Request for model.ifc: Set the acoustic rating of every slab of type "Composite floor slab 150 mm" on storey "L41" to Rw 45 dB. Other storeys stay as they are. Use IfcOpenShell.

First a look at what the model holds.

```python
import ifcopenshell
import ifcopenshell.util.element

model = ifcopenshell.open("model.ifc")
print(model.schema)
storey = next(s for s in model.by_type("IfcBuildingStorey") if s.Name == "L41")
slabs = [e for e in ifcopenshell.util.element.get_decomposition(storey) if e.is_a("IfcSlab")]
seen = {}
for e in slabs:
    element_type = ifcopenshell.util.element.get_type(e)
    key = (element_type.Name if element_type != e and element_type else None, ifcopenshell.util.element.get_pset(e, "Pset_SlabCommon", "AcousticRating"))
    seen[key] = seen.get(key, 0) + 1
for (name, value), count in sorted(seen.items(), key=str):
    print(count, "x", name, "|", value)
```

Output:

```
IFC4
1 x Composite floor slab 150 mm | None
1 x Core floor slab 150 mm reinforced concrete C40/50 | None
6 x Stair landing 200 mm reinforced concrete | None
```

```python
import ifcopenshell
import ifcopenshell.api.pset
import ifcopenshell.util.element

model = ifcopenshell.open("model.ifc")

storey = next(s for s in model.by_type("IfcBuildingStorey") if s.Name == "L41")
slabs = [e for e in ifcopenshell.util.element.get_decomposition(storey) if e.is_a("IfcSlab")]

count = 0
for e in slabs:
    element_type = ifcopenshell.util.element.get_type(e)
    if element_type in (None, e) or element_type.Name != "Composite floor slab 150 mm":
        continue
    found = ifcopenshell.util.element.get_pset(e, "Pset_SlabCommon", should_inherit=False)
    if found:
        pset = model.by_id(found["id"])
        if len(ifcopenshell.util.element.get_elements_by_pset(pset)) > 1:
            pset = ifcopenshell.api.pset.unshare_pset(model, products=[e], pset=pset)[0]
    else:
        pset = ifcopenshell.api.pset.add_pset(model, product=e, name="Pset_SlabCommon")
    ifcopenshell.api.pset.edit_pset(model, pset=pset, properties={"AcousticRating": "Rw 45 dB"})
    count += 1

print(count, "slabs updated")

model.write("model_rev.ifc")
```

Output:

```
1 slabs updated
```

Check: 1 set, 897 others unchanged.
